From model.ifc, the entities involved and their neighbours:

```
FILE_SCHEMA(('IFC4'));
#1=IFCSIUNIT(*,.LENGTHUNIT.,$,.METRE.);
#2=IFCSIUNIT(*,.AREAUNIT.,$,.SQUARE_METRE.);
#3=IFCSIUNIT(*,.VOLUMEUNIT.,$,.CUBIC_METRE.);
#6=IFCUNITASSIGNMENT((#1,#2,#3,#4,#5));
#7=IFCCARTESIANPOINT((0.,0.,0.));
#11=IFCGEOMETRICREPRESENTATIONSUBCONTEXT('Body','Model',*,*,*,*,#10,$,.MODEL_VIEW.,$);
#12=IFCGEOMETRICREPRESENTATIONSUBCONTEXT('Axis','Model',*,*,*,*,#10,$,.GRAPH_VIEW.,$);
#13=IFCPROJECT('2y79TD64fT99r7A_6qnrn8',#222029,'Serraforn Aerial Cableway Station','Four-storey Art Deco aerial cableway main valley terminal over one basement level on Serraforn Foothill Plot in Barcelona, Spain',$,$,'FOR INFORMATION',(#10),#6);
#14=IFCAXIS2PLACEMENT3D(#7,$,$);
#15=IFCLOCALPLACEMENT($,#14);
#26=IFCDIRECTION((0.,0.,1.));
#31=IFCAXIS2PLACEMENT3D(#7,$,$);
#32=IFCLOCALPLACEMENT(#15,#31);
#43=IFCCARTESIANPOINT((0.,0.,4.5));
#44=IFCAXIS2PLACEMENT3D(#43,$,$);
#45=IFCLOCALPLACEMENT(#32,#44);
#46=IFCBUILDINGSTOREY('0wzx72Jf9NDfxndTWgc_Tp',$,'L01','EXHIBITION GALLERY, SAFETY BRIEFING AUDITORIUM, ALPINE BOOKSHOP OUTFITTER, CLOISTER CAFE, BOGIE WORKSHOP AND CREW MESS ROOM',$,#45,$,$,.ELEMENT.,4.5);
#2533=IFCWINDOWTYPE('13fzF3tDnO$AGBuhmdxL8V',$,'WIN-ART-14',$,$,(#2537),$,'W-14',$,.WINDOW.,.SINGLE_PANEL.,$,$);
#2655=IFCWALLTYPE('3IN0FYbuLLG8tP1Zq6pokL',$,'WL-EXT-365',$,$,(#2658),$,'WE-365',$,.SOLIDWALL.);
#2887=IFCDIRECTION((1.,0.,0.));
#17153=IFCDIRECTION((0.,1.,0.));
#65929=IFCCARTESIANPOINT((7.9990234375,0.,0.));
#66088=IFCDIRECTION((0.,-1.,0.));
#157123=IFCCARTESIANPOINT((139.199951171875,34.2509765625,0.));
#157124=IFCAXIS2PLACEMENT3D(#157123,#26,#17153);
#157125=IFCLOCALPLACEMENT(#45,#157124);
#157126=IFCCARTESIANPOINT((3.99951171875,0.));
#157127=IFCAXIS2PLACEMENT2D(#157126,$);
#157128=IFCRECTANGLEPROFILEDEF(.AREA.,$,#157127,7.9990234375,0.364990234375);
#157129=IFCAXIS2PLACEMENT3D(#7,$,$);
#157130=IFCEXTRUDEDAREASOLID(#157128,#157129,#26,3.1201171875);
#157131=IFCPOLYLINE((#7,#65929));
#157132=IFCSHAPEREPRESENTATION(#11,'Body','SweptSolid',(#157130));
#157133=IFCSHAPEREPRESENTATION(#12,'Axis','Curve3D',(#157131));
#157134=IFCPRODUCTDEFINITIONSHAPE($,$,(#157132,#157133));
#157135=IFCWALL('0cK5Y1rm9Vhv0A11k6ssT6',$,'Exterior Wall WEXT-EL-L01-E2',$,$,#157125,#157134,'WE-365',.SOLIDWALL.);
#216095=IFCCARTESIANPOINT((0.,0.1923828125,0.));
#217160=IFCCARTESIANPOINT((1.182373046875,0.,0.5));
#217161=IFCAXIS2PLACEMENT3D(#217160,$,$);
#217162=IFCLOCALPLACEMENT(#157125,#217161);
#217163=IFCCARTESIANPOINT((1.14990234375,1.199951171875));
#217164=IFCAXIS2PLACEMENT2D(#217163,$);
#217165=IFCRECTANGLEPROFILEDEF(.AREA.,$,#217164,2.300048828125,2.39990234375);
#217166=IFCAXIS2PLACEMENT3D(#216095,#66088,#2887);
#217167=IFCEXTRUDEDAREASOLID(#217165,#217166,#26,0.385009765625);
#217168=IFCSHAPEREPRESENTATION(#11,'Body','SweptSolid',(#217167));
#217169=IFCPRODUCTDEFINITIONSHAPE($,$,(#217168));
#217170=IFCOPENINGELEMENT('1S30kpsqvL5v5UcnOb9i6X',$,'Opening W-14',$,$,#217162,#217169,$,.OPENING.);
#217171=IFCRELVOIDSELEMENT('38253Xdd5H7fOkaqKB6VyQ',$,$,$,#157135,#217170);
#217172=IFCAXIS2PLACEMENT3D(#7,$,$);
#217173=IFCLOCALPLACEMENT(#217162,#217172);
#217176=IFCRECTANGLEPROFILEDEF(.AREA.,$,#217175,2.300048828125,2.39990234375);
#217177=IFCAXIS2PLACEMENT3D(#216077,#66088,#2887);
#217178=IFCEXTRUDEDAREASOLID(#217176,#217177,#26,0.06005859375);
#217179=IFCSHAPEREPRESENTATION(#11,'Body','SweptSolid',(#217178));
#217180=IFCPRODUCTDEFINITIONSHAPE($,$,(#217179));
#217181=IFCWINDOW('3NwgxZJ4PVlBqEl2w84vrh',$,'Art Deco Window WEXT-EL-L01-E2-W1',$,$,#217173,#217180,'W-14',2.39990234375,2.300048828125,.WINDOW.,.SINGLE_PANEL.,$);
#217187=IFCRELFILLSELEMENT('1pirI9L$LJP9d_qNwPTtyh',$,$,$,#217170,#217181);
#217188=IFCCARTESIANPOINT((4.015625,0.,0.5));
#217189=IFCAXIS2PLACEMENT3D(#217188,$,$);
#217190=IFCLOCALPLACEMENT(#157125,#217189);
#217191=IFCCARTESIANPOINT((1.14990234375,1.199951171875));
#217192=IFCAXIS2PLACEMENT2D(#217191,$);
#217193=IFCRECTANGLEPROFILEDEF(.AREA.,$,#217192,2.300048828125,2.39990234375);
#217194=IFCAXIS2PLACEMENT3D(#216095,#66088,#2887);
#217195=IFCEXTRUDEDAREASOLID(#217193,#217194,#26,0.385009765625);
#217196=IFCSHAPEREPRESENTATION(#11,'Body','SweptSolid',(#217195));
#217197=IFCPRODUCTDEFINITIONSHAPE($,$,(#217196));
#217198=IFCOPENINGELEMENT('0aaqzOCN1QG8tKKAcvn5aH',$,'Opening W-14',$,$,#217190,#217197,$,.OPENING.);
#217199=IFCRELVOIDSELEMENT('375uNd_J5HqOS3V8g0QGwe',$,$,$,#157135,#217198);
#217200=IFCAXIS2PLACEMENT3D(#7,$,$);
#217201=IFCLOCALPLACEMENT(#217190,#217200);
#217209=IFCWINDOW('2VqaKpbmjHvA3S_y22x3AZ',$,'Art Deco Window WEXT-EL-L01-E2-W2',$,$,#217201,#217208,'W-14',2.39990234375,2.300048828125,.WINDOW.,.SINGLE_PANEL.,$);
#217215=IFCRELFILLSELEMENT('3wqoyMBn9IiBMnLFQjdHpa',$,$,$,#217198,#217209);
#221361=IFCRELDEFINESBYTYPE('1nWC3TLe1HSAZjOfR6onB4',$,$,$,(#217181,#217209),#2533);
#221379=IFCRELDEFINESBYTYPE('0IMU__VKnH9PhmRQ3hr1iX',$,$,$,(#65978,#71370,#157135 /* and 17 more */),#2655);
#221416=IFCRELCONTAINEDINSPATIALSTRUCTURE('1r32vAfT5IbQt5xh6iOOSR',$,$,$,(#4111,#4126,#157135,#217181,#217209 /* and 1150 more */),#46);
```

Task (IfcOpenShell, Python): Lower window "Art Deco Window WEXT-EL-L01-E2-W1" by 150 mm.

```python
import numpy as np
import ifcopenshell
import ifcopenshell.api.geometry
import ifcopenshell.util.placement
import ifcopenshell.util.unit

model = ifcopenshell.open("model.ifc")
unit_scale = ifcopenshell.util.unit.calculate_unit_scale(model)

window = model.by_guid("3NwgxZJ4PVlBqEl2w84vrh")
opening = window.FillsVoids[0].RelatingOpeningElement
dz = -0.15

shift = np.array([0.0, 0.0, dz])
# The window is placed relative to its opening, so it follows when the opening moves.
matrix = ifcopenshell.util.placement.get_local_placement(opening.ObjectPlacement)
matrix[:3, 3] += shift
ifcopenshell.api.geometry.edit_object_placement(
    model, product=opening, matrix=matrix, is_si=False, should_transform_children=True
)

print(f"moved by {dz * unit_scale:+.3f} m")

model.write("model_rev.ifc")
```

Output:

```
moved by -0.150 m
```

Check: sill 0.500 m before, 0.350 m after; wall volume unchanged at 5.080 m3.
